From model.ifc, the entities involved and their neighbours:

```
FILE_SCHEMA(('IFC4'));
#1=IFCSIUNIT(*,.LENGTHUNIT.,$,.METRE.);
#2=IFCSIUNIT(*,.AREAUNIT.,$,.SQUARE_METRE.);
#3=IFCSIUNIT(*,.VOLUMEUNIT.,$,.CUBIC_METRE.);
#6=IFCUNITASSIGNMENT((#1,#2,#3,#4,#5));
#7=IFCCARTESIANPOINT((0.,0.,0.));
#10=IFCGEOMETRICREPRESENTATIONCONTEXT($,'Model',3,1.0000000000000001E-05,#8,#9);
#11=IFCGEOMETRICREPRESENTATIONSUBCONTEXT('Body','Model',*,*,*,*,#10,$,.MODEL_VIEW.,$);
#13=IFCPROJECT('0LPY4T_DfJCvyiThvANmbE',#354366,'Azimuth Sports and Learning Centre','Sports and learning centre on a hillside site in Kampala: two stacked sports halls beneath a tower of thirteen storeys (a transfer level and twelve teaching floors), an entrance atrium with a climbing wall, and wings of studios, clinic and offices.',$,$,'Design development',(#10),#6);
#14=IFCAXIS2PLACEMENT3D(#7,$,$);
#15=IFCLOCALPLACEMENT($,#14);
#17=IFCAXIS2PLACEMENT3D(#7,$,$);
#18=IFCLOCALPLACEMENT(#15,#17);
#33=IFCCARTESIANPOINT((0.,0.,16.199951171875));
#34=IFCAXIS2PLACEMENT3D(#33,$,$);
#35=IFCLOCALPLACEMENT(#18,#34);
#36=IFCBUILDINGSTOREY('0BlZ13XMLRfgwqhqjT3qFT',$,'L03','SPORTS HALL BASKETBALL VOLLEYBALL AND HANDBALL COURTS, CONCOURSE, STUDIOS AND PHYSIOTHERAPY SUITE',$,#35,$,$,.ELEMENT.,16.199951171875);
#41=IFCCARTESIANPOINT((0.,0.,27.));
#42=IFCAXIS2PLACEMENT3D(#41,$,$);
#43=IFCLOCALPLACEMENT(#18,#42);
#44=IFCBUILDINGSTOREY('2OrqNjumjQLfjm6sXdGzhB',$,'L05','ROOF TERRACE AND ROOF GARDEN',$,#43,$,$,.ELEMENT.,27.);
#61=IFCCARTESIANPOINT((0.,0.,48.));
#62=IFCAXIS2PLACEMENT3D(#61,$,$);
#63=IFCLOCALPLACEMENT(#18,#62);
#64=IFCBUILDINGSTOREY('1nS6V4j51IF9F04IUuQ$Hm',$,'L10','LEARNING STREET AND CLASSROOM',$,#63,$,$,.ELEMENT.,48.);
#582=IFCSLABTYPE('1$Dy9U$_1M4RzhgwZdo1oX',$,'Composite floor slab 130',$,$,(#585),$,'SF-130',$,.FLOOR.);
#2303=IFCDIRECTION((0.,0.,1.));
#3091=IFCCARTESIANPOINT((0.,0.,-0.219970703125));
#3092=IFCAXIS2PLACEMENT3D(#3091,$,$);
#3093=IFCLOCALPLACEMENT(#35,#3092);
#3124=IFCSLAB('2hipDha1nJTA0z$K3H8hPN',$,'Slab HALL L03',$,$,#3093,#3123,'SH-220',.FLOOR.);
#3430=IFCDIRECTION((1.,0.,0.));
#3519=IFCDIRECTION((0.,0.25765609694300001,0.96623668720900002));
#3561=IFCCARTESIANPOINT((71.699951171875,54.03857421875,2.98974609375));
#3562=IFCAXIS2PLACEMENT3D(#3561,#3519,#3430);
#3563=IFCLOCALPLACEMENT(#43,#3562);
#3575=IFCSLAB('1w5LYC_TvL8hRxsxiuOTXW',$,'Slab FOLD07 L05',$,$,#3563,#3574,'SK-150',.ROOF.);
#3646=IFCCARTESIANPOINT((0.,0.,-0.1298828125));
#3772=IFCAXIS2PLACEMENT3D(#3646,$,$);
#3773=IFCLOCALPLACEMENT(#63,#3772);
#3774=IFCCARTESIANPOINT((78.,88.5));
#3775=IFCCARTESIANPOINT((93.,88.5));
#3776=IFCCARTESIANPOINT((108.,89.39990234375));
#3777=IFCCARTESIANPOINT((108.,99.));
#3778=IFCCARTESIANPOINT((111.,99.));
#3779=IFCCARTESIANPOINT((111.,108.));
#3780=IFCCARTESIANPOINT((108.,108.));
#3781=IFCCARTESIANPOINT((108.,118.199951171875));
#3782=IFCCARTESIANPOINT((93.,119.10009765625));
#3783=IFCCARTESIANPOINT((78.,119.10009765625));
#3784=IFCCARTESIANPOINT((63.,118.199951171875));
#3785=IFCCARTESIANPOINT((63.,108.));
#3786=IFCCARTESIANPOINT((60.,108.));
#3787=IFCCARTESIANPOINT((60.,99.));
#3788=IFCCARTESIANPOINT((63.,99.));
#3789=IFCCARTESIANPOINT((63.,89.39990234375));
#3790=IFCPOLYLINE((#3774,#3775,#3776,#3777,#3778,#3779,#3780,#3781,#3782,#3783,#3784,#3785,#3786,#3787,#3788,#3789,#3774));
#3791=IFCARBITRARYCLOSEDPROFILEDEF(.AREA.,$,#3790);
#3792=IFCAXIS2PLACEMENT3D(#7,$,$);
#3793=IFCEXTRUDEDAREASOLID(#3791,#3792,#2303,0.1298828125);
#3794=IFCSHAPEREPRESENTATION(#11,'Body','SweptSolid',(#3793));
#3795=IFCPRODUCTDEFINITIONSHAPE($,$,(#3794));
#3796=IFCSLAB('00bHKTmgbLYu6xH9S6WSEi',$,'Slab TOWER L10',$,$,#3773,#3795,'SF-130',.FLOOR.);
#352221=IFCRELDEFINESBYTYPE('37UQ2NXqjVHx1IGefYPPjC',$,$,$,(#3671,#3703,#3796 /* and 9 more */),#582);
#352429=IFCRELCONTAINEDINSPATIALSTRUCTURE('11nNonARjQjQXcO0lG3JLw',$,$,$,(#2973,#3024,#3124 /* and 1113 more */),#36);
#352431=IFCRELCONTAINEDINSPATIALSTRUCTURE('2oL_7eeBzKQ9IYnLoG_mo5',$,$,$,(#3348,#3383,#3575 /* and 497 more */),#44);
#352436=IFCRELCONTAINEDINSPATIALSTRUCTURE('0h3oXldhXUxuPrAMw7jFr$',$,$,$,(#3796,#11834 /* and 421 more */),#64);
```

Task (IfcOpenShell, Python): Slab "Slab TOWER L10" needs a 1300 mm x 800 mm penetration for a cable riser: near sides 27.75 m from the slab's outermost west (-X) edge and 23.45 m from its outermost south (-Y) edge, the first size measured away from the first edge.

```python
import numpy as np
import ifcopenshell
import ifcopenshell.api.feature
import ifcopenshell.api.geometry
import ifcopenshell.api.root
import ifcopenshell.geom
import ifcopenshell.util.placement
import ifcopenshell.util.representation
import ifcopenshell.util.shape
import ifcopenshell.util.unit

model = ifcopenshell.open("model.ifc")
unit_scale = ifcopenshell.util.unit.calculate_unit_scale(model)
settings = ifcopenshell.geom.settings()


def volume(element):
    """Net volume in cubic metres, openings subtracted."""
    shape = ifcopenshell.geom.create_shape(settings, element)
    return ifcopenshell.util.shape.get_volume(shape.geometry)


slab = model.by_guid("00bHKTmgbLYu6xH9S6WSEi")
before = volume(slab)

# Extent in the slab's own axes, in metres. The edges named are its -X and -Y sides.
slab_shape = ifcopenshell.geom.create_shape(settings, slab)
vertices = ifcopenshell.util.shape.get_vertices(slab_shape.geometry)
x_min, y_min, bottom = vertices.min(axis=0)
top = vertices[:, 2].max()

opening = ifcopenshell.api.root.create_entity(model, ifc_class="IfcOpeningElement", name="Cable riser opening", predefined_type="OPENING")
context = ifcopenshell.util.representation.get_context(model, "Model", "Body", "MODEL_VIEW")
width, depth = 1.3, 0.8
outline = [(0.0, 0.0), (width, 0.0), (width, depth), (0.0, depth), (0.0, 0.0)]
# Overshoot both faces by 50 mm so the cut is clean.
shape = ifcopenshell.api.geometry.add_slab_representation(
    model, context=context, depth=top - bottom + 0.1, polyline=outline
)
ifcopenshell.api.geometry.assign_representation(model, product=opening, representation=shape)

matrix = ifcopenshell.util.placement.get_local_placement(slab.ObjectPlacement)
matrix[:, 3] = matrix @ np.append(np.array([x_min + 27.75, y_min + 23.45, bottom - 0.05]) / unit_scale, 1.0)
ifcopenshell.api.geometry.edit_object_placement(model, product=opening, matrix=matrix, is_si=False)
ifcopenshell.api.feature.add_feature(model, feature=opening, element=slab)

after = volume(slab)

print(f"slab volume {before:.3f} -> {after:.3f} m3")

model.write("model_v2.ifc")
```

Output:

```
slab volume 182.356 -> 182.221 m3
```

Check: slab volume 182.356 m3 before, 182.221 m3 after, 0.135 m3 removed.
